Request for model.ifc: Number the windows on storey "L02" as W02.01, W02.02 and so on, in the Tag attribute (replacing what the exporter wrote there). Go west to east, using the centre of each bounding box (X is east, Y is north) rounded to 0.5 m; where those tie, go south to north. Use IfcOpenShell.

First a look at what the model holds.

```python
import ifcopenshell
import ifcopenshell.util.element
import ifcopenshell.util.placement

model = ifcopenshell.open("model.ifc")
print(model.schema)
storey = next(s for s in model.by_type("IfcBuildingStorey") if s.Name == "L02")
windows = [e for e in ifcopenshell.util.element.get_decomposition(storey) if e.is_a("IfcWindow")]
for e in sorted(windows, key=lambda e: e.id()):
    origin = ifcopenshell.util.placement.get_local_placement(e.ObjectPlacement)[:3, 3]
    print(e.id(), e.Tag, e.Name, origin.round(2) + 0.0, sep=" | ")
```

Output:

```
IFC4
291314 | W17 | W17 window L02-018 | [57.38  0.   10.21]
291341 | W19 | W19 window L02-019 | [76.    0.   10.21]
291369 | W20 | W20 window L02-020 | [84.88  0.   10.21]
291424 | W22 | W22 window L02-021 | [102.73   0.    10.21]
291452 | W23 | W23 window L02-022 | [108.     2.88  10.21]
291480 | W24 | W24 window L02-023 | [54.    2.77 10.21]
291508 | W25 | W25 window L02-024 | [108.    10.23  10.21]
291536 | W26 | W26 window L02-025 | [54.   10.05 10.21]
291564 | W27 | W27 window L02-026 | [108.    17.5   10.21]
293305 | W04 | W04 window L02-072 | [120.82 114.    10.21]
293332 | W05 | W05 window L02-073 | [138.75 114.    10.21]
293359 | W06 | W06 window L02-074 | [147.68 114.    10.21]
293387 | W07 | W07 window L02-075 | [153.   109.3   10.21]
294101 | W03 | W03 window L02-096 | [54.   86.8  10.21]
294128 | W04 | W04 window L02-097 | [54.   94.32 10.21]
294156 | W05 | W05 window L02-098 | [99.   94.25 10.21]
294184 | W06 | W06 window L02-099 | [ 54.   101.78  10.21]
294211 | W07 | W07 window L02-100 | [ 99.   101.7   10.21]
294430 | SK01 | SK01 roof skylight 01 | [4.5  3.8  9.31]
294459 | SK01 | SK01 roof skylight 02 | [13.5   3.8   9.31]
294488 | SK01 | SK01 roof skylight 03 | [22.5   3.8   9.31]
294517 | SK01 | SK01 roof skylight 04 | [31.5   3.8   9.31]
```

```python
import ifcopenshell
import ifcopenshell.geom
import ifcopenshell.util.element
import ifcopenshell.util.shape

model = ifcopenshell.open("model.ifc")
settings = ifcopenshell.geom.settings()
settings.set("use-world-coords", True)


def centre(element):
    shape = ifcopenshell.geom.create_shape(settings, element)
    return ifcopenshell.util.shape.get_bbox_centroid(shape.geometry)


storey = next(s for s in model.by_type("IfcBuildingStorey") if s.Name == "L02")
windows = [e for e in ifcopenshell.util.element.get_decomposition(storey) if e.is_a("IfcWindow")]

# Insertion points can sit at a corner or the storey origin, so sort by the geometry (in metres).
centres = {e: centre(e) for e in windows}
windows.sort(key=lambda e: (round(centres[e][0] / 0.5), centres[e][1]))

for i, e in enumerate(windows, start=1):
    number = f"W02.{i:02d}"
    e.Tag = number
    print(e.id(), number)

model.write("model_v2.ifc")
```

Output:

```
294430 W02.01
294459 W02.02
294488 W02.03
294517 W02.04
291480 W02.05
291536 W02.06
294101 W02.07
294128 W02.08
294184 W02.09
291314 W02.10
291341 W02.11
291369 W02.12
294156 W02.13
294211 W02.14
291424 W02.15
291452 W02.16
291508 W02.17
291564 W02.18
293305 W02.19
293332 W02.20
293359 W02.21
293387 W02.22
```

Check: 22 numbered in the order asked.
